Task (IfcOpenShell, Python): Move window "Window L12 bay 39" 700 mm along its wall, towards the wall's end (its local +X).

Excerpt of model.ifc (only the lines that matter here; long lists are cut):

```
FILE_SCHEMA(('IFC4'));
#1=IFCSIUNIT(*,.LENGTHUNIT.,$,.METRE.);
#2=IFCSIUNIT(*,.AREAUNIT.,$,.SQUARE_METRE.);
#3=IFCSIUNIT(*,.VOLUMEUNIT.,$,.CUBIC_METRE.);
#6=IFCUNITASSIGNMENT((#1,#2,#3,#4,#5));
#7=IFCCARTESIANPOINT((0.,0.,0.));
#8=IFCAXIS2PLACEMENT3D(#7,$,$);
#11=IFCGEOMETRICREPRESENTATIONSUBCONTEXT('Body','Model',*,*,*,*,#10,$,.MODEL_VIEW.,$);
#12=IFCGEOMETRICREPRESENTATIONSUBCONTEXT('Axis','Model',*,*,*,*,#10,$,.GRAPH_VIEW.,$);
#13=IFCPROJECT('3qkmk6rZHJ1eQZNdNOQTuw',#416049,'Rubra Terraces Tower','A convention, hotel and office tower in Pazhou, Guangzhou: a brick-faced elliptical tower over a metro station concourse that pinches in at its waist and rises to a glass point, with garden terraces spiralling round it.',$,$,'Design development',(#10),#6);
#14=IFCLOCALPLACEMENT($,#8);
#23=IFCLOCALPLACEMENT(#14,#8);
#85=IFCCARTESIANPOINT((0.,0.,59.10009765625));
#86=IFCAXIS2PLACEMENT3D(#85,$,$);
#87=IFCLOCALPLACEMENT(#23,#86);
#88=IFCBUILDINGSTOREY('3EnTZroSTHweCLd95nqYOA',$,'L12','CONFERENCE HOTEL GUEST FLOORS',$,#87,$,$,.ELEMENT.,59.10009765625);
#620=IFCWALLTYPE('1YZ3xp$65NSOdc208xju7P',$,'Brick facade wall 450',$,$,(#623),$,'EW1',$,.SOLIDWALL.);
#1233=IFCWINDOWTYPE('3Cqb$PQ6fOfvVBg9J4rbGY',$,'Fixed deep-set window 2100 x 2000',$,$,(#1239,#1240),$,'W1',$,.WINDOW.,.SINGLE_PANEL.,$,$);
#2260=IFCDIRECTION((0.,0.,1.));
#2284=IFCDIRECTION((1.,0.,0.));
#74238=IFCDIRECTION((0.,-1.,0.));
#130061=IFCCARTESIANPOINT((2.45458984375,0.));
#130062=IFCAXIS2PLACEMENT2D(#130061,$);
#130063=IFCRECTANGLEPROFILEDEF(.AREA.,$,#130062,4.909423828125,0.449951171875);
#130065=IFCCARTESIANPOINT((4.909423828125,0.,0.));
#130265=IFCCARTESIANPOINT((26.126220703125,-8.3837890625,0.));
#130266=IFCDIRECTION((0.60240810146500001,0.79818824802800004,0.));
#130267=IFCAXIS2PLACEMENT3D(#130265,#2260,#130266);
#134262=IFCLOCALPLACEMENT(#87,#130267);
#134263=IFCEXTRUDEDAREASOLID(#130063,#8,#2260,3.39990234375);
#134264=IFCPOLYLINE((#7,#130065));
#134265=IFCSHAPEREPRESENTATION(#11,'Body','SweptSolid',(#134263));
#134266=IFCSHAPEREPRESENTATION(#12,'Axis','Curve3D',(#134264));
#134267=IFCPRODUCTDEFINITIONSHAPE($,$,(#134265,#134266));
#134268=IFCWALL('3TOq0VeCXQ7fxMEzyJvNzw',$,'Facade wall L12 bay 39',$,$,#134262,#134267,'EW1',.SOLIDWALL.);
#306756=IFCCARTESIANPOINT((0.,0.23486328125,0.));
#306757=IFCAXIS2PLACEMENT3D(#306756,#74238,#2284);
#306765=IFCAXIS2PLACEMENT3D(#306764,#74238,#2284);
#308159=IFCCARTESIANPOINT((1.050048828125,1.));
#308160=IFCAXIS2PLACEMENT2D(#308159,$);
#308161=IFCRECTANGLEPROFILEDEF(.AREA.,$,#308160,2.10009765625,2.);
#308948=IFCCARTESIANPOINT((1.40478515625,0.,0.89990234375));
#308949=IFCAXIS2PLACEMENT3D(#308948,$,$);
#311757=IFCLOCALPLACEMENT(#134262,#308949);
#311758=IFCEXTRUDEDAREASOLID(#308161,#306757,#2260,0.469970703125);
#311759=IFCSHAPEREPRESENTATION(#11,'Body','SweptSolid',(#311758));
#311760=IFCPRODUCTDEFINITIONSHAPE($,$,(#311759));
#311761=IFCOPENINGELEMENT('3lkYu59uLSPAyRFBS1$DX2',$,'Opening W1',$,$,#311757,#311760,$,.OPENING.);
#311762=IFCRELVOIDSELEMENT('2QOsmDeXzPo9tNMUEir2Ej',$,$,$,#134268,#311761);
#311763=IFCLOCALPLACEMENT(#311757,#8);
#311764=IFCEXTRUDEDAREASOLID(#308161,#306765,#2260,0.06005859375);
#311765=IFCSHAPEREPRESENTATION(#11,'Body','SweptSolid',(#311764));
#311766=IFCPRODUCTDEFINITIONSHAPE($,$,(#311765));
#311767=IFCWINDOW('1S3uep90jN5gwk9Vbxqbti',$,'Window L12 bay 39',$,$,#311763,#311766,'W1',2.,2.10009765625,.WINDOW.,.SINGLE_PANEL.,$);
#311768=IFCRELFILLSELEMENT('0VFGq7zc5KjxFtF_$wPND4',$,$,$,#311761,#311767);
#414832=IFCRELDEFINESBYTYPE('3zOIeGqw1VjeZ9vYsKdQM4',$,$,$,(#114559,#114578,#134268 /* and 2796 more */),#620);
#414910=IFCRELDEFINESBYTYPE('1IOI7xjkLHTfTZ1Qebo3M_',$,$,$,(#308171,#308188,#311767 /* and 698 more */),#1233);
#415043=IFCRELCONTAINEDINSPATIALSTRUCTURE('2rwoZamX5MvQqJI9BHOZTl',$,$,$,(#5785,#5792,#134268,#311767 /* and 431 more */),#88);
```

```python
import ifcopenshell
import ifcopenshell.api.geometry
import ifcopenshell.util.placement
import ifcopenshell.util.unit

model = ifcopenshell.open("model.ifc")
unit_scale = ifcopenshell.util.unit.calculate_unit_scale(model)

window = model.by_guid("1S3uep90jN5gwk9Vbxqbti")
opening = window.FillsVoids[0].RelatingOpeningElement
wall = opening.VoidsElements[0].RelatingBuildingElement

wall_matrix = ifcopenshell.util.placement.get_local_placement(wall.ObjectPlacement)
shift = wall_matrix[:3, 0] * 0.7 / unit_scale
before = ifcopenshell.util.placement.get_local_placement(window.ObjectPlacement)[:3, 3].copy()

# The window is placed relative to its opening, so it follows when the opening moves.
matrix = ifcopenshell.util.placement.get_local_placement(opening.ObjectPlacement)
matrix[:3, 3] += shift
ifcopenshell.api.geometry.edit_object_placement(
    model, product=opening, matrix=matrix, is_si=False, should_transform_children=True
)

after = ifcopenshell.util.placement.get_local_placement(window.ObjectPlacement)[:3, 3]
print("window moved by", (after - before).round(3) + 0.0)

model.write("model_v2.ifc")
```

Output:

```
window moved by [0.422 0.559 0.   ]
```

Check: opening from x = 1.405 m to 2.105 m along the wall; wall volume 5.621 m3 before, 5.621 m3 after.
